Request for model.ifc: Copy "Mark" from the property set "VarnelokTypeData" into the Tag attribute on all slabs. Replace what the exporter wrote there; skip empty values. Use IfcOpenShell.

First a look at what the model holds.

```python
import ifcopenshell
import ifcopenshell.util.element

model = ifcopenshell.open("model.ifc")
print(model.schema)
slabs = model.by_type("IfcSlab")
print(len(slabs), "slabs")
for e in slabs[:8]:
    source = ifcopenshell.util.element.get_pset(e, "VarnelokTypeData", "Mark")
    target = e.Tag
    print(e.id(), repr(source), repr(target), sep=" | ")
```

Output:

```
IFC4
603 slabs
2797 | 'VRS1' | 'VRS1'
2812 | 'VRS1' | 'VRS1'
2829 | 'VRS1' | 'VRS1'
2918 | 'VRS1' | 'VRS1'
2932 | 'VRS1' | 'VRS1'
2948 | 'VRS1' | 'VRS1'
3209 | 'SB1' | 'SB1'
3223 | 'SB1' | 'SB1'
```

```python
import ifcopenshell
import ifcopenshell.util.element

model = ifcopenshell.open("model.ifc")

count = 0
for e in model.by_type("IfcSlab"):
    value = ifcopenshell.util.element.get_pset(e, "VarnelokTypeData", "Mark")
    current = e.Tag
    if not value or not value.strip() or current == value:
        continue
    e.Tag = value
    count += 1

print(count, "slabs updated")

model.write("model-out.ifc")
```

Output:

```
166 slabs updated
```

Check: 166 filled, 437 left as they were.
